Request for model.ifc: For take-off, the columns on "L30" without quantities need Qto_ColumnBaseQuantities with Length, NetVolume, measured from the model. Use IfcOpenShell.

First a look at what the model holds.

```python
import ifcopenshell
import ifcopenshell.util.element
import ifcopenshell.util.unit

model = ifcopenshell.open("model.ifc")
print(model.schema)
for unit_type in ("LENGTHUNIT", "AREAUNIT", "VOLUMEUNIT"):
    print(unit_type, ifcopenshell.util.unit.calculate_unit_scale(model, unit_type))
storey = next(s for s in model.by_type("IfcBuildingStorey") if s.Name == "L30")
columns = [e for e in ifcopenshell.util.element.get_decomposition(storey) if e.is_a("IfcColumn")]
for e in sorted(columns, key=lambda e: e.id()):
    print(e.id(), e.is_a(), e.Name, list(ifcopenshell.util.element.get_psets(e, qtos_only=True)), sep=" | ")
```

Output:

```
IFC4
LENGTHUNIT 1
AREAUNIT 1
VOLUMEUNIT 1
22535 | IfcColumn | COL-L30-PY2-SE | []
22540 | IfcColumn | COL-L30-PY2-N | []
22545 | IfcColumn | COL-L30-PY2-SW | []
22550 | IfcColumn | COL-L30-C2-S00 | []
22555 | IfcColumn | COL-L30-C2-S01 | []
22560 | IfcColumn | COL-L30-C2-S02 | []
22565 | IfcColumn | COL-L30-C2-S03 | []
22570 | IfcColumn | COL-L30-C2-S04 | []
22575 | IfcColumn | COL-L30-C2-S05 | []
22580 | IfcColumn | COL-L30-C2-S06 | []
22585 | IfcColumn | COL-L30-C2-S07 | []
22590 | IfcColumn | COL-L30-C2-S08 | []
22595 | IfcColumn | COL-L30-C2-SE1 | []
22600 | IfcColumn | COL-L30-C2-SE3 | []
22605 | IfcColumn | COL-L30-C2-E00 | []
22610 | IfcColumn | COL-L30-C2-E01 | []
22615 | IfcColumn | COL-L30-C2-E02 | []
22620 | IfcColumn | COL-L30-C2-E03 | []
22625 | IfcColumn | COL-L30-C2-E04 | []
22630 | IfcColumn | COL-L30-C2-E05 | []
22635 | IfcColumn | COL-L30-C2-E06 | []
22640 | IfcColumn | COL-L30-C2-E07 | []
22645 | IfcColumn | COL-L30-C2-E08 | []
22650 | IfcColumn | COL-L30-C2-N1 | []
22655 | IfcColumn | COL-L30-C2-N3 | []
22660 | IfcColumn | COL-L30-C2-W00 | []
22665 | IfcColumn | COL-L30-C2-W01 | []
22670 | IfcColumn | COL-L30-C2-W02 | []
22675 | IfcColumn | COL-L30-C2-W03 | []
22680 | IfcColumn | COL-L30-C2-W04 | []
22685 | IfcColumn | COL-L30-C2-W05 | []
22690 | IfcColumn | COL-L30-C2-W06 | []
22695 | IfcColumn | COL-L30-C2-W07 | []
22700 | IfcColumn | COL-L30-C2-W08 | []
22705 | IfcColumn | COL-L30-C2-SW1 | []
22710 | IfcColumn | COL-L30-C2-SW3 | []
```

```python
import ifcopenshell
import ifcopenshell.api.pset
import ifcopenshell.geom
import ifcopenshell.util.element
import ifcopenshell.util.shape
import ifcopenshell.util.unit

model = ifcopenshell.open("model.ifc")
unit_scale = ifcopenshell.util.unit.calculate_unit_scale(model)
volume_scale = ifcopenshell.util.unit.calculate_unit_scale(model, "VOLUMEUNIT")
settings = ifcopenshell.geom.settings()

storey = next(s for s in model.by_type("IfcBuildingStorey") if s.Name == "L30")
columns = [e for e in ifcopenshell.util.element.get_decomposition(storey) if e.is_a("IfcColumn")]

for e in sorted(columns, key=lambda e: e.id()):
    if ifcopenshell.util.element.get_psets(e, qtos_only=True, should_inherit=False):
        continue
    # Geometry comes back in metres, in the element's own axes.
    shape = ifcopenshell.geom.create_shape(settings, e)
    values = {
        "Length": ifcopenshell.util.shape.get_z(shape.geometry) / unit_scale,
        "NetVolume": ifcopenshell.util.shape.get_volume(shape.geometry) / volume_scale,
    }
    qto = ifcopenshell.api.pset.add_qto(model, product=e, name="Qto_ColumnBaseQuantities")
    ifcopenshell.api.pset.edit_qto(model, qto=qto, properties=values)
    print(e.id(), {k: round(v, 3) for k, v in values.items()})

model.write("model_rev.ifc")
```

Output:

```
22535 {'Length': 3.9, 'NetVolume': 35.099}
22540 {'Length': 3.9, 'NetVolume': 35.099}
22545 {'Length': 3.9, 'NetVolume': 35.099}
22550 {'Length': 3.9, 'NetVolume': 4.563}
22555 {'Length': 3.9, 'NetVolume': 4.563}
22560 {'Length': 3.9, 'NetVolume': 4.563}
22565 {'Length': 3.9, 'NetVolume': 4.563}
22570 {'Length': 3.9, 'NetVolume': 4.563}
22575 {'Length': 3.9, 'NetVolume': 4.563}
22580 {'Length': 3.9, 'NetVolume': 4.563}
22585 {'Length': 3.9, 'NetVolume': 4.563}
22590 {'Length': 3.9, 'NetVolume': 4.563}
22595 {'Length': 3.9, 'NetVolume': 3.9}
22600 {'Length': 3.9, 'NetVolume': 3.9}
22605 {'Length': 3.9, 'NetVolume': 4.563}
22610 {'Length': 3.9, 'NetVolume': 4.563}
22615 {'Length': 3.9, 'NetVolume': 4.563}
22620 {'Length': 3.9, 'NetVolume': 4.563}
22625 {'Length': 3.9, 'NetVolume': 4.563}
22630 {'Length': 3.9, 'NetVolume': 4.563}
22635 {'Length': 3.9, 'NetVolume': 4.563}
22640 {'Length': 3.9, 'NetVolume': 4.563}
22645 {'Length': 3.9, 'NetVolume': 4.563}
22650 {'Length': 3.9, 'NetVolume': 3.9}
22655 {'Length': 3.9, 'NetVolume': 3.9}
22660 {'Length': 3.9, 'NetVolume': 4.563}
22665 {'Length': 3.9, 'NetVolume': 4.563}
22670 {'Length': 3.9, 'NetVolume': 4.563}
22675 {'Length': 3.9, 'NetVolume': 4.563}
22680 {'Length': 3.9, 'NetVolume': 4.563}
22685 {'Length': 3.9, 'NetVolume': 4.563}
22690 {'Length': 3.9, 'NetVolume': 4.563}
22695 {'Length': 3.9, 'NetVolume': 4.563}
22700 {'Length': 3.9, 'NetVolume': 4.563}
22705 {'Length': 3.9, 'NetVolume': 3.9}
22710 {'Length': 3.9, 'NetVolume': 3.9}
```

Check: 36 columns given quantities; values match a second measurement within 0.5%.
